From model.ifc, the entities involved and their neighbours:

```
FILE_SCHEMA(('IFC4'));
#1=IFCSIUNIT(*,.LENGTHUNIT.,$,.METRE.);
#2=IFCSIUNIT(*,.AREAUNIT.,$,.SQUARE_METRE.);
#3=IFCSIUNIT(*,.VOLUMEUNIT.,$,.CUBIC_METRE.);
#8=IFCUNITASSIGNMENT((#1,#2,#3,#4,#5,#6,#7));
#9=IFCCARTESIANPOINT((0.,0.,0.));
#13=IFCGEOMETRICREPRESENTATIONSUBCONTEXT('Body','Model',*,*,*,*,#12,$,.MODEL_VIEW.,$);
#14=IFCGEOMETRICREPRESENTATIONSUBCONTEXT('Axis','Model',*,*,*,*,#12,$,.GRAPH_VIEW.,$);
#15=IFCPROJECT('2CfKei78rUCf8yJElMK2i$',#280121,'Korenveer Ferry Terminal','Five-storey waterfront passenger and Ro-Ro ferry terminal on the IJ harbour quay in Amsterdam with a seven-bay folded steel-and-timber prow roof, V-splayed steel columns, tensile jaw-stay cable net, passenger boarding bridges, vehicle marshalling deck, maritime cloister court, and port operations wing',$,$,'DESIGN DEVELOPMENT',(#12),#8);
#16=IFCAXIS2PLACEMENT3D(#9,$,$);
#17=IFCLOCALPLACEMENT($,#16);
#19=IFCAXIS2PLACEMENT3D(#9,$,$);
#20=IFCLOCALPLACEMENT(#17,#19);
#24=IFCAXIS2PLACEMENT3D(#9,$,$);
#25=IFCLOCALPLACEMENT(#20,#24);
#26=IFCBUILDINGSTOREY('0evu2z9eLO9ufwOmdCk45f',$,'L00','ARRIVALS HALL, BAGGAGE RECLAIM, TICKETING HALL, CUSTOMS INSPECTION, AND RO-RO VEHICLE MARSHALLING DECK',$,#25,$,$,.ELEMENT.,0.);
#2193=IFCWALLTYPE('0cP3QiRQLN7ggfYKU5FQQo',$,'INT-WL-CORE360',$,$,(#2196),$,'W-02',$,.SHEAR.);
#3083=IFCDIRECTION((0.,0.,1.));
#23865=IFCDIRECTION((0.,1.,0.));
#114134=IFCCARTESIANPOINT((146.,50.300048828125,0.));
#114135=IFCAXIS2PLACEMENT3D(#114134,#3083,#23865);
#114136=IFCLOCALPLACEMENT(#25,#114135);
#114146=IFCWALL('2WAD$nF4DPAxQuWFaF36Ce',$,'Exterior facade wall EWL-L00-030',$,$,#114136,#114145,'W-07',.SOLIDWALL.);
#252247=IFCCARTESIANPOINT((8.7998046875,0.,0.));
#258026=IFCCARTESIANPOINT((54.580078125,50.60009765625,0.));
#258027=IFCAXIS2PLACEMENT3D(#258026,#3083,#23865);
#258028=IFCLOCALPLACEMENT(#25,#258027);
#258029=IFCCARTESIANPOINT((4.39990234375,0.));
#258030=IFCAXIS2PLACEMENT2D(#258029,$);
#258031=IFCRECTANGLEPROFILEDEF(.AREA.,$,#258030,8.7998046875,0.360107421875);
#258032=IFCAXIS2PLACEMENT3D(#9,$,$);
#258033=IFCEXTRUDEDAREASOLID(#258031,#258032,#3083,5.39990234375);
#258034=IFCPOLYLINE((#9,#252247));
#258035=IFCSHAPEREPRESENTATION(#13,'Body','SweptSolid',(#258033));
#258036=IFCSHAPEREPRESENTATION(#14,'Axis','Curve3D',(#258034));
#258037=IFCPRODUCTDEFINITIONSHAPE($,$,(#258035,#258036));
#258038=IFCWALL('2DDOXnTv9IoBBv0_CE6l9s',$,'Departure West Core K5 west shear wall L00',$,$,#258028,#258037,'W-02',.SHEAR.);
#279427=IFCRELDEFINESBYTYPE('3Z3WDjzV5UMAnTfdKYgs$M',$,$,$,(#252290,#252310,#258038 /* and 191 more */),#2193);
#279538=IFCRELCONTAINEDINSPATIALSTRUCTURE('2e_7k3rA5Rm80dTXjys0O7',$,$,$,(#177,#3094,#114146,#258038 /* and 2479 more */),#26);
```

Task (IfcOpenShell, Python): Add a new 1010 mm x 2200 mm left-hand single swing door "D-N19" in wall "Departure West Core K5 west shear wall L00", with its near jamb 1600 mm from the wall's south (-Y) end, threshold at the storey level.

```python
import numpy as np
import ifcopenshell
import ifcopenshell.api.feature
import ifcopenshell.api.geometry
import ifcopenshell.api.root
import ifcopenshell.api.spatial
import ifcopenshell.geom
import ifcopenshell.util.element
import ifcopenshell.util.placement
import ifcopenshell.util.representation
import ifcopenshell.util.shape
import ifcopenshell.util.unit

model = ifcopenshell.open("model.ifc")
unit_scale = ifcopenshell.util.unit.calculate_unit_scale(model)
settings = ifcopenshell.geom.settings()


def volume(element):
    """Net volume in cubic metres, openings subtracted."""
    shape = ifcopenshell.geom.create_shape(settings, element)
    return ifcopenshell.util.shape.get_volume(shape.geometry)


wall = model.by_guid("2DDOXnTv9IoBBv0_CE6l9s")
storey = ifcopenshell.util.element.get_container(wall, ifc_class="IfcBuildingStorey")
context = ifcopenshell.util.representation.get_context(model, "Model", "Body", "MODEL_VIEW")
before = volume(wall)

width, height, from_end, sill = 1.01, 2.2, 1.6, 0.0  # metres

# The wall runs along its own X axis, and the end named is its -X end.
wall_shape = ifcopenshell.geom.create_shape(settings, wall)
x, y, z = ifcopenshell.util.shape.get_vertices(wall_shape.geometry).T
start = x.min() + from_end
face, thickness = float(y.min()), float(y.max() - y.min())
wall_matrix = ifcopenshell.util.placement.get_local_placement(wall.ObjectPlacement)
level = ifcopenshell.util.placement.get_local_placement(storey.ObjectPlacement)[2, 3]


def in_wall(x, y):
    """Placement at x, y metres in the wall's axes, at sill height."""
    matrix = wall_matrix.copy()
    matrix[:, 3] = wall_matrix @ np.array([x / unit_scale, y / unit_scale, 0.0, 1.0])
    matrix[2, 3] = level + sill / unit_scale
    return matrix


# Opening: a box that overshoots both wall faces by 50 mm.
opening = ifcopenshell.api.root.create_entity(model, ifc_class="IfcOpeningElement", predefined_type="OPENING")
box = ifcopenshell.api.geometry.add_wall_representation(
    model, context=context, length=width, height=height, thickness=thickness + 0.1
)
ifcopenshell.api.geometry.assign_representation(model, product=opening, representation=box)
ifcopenshell.api.geometry.edit_object_placement(model, product=opening, matrix=in_wall(start, face - 0.05), is_si=False)
ifcopenshell.api.feature.add_feature(model, feature=opening, element=wall)

door = ifcopenshell.api.root.create_entity(model, ifc_class="IfcDoor", name="D-N19", predefined_type="DOOR")
door.OverallWidth, door.OverallHeight = width / unit_scale, height / unit_scale
door.OperationType = "SINGLE_SWING_LEFT"
body = ifcopenshell.api.geometry.add_door_representation(
    model,
    context=context,
    overall_width=door.OverallWidth,
    overall_height=door.OverallHeight,
    operation_type="SINGLE_SWING_LEFT",
    lining_properties={"LiningDepth": thickness / unit_scale, "ThresholdDepth": thickness / unit_scale},
)
ifcopenshell.api.geometry.assign_representation(model, product=door, representation=body)
ifcopenshell.api.spatial.assign_container(model, products=[door], relating_structure=storey)
ifcopenshell.api.feature.add_filling(model, opening=opening, element=door)

# The lining spans the wall, so the door starts at the wall face.
ifcopenshell.api.geometry.edit_object_placement(model, product=door, matrix=in_wall(start, face), is_si=False)

after = volume(wall)

print(f"wall volume {before:.3f} -> {after:.3f} m3")

model.write("model_edited.ifc")
```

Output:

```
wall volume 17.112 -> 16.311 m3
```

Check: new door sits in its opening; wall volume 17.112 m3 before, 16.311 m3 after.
